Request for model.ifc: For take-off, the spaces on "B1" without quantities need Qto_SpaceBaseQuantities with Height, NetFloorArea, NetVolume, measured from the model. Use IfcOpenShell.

First a look at what the model holds.

```python
import ifcopenshell
import ifcopenshell.util.element
import ifcopenshell.util.unit

model = ifcopenshell.open("model.ifc")
print(model.schema)
for unit_type in ("LENGTHUNIT", "AREAUNIT", "VOLUMEUNIT"):
    print(unit_type, ifcopenshell.util.unit.calculate_unit_scale(model, unit_type))
storey = next(s for s in model.by_type("IfcBuildingStorey") if s.Name == "B1")
spaces = [e for e in ifcopenshell.util.element.get_decomposition(storey) if e.is_a("IfcSpace")]
for e in sorted(spaces, key=lambda e: e.id()):
    print(e.id(), e.is_a(), e.Name, list(ifcopenshell.util.element.get_psets(e, qtos_only=True)), sep=" | ")
```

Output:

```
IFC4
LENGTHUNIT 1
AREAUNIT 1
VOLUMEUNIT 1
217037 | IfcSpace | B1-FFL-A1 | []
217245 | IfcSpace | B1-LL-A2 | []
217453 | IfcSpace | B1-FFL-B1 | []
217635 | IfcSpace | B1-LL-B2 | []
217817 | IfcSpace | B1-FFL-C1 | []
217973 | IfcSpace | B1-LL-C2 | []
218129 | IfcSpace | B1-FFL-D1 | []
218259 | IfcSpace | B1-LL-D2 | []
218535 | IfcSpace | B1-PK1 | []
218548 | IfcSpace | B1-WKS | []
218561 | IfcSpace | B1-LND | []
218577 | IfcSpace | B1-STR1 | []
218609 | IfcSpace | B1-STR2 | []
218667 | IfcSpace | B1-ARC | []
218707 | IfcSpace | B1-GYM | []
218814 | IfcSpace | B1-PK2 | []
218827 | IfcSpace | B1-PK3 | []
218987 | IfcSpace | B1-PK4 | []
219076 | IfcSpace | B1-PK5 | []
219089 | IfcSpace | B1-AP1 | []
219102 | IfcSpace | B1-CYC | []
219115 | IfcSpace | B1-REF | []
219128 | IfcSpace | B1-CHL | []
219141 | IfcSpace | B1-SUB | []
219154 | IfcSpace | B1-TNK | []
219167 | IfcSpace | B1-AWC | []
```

```python
import ifcopenshell
import ifcopenshell.api.pset
import ifcopenshell.geom
import ifcopenshell.util.element
import ifcopenshell.util.shape
import ifcopenshell.util.unit

model = ifcopenshell.open("model.ifc")
unit_scale = ifcopenshell.util.unit.calculate_unit_scale(model)
area_scale = ifcopenshell.util.unit.calculate_unit_scale(model, "AREAUNIT")
volume_scale = ifcopenshell.util.unit.calculate_unit_scale(model, "VOLUMEUNIT")
settings = ifcopenshell.geom.settings()

storey = next(s for s in model.by_type("IfcBuildingStorey") if s.Name == "B1")
spaces = [e for e in ifcopenshell.util.element.get_decomposition(storey) if e.is_a("IfcSpace")]

for e in sorted(spaces, key=lambda e: e.id()):
    if ifcopenshell.util.element.get_psets(e, qtos_only=True, should_inherit=False):
        continue
    # Geometry comes back in metres, in the element's own axes.
    shape = ifcopenshell.geom.create_shape(settings, e)
    values = {
        "Height": ifcopenshell.util.shape.get_z(shape.geometry) / unit_scale,
        "NetFloorArea": ifcopenshell.util.shape.get_footprint_area(shape.geometry) / area_scale,
        "NetVolume": ifcopenshell.util.shape.get_volume(shape.geometry) / volume_scale,
    }
    qto = ifcopenshell.api.pset.add_qto(model, product=e, name="Qto_SpaceBaseQuantities")
    ifcopenshell.api.pset.edit_qto(model, qto=qto, properties=values)
    print(e.id(), {k: round(v, 3) for k, v in values.items()})

model.write("model_updated.ifc")
```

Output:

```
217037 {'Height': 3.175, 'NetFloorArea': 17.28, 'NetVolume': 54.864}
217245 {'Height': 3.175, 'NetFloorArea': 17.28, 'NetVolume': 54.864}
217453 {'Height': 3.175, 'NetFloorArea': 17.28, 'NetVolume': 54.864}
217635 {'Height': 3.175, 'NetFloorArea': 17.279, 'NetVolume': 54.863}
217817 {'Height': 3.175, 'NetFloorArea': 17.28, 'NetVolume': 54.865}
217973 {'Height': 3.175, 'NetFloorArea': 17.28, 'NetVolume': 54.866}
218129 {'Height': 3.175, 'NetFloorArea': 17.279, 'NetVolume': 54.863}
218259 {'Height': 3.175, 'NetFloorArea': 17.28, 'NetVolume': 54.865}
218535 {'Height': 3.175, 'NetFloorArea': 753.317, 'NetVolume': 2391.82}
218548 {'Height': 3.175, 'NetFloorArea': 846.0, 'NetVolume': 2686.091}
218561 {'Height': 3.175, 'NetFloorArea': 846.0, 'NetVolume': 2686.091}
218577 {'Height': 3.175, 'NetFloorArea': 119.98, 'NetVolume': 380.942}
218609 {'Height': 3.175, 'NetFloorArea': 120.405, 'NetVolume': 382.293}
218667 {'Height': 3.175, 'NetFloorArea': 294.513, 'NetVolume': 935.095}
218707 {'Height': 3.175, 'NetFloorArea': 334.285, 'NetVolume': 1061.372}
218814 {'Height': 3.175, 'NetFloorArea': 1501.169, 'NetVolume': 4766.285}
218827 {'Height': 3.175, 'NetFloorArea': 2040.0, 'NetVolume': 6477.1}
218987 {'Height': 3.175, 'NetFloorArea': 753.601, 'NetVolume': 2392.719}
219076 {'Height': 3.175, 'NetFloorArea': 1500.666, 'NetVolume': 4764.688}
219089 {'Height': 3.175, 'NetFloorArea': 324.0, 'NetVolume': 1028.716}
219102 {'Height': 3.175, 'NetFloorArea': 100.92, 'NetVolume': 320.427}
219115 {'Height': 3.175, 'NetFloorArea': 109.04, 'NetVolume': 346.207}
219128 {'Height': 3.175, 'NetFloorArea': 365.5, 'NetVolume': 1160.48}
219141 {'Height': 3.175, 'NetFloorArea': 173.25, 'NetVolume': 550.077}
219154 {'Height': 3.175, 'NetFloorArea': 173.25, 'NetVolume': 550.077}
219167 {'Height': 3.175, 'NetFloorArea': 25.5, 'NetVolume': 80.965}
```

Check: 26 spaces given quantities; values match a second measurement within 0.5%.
